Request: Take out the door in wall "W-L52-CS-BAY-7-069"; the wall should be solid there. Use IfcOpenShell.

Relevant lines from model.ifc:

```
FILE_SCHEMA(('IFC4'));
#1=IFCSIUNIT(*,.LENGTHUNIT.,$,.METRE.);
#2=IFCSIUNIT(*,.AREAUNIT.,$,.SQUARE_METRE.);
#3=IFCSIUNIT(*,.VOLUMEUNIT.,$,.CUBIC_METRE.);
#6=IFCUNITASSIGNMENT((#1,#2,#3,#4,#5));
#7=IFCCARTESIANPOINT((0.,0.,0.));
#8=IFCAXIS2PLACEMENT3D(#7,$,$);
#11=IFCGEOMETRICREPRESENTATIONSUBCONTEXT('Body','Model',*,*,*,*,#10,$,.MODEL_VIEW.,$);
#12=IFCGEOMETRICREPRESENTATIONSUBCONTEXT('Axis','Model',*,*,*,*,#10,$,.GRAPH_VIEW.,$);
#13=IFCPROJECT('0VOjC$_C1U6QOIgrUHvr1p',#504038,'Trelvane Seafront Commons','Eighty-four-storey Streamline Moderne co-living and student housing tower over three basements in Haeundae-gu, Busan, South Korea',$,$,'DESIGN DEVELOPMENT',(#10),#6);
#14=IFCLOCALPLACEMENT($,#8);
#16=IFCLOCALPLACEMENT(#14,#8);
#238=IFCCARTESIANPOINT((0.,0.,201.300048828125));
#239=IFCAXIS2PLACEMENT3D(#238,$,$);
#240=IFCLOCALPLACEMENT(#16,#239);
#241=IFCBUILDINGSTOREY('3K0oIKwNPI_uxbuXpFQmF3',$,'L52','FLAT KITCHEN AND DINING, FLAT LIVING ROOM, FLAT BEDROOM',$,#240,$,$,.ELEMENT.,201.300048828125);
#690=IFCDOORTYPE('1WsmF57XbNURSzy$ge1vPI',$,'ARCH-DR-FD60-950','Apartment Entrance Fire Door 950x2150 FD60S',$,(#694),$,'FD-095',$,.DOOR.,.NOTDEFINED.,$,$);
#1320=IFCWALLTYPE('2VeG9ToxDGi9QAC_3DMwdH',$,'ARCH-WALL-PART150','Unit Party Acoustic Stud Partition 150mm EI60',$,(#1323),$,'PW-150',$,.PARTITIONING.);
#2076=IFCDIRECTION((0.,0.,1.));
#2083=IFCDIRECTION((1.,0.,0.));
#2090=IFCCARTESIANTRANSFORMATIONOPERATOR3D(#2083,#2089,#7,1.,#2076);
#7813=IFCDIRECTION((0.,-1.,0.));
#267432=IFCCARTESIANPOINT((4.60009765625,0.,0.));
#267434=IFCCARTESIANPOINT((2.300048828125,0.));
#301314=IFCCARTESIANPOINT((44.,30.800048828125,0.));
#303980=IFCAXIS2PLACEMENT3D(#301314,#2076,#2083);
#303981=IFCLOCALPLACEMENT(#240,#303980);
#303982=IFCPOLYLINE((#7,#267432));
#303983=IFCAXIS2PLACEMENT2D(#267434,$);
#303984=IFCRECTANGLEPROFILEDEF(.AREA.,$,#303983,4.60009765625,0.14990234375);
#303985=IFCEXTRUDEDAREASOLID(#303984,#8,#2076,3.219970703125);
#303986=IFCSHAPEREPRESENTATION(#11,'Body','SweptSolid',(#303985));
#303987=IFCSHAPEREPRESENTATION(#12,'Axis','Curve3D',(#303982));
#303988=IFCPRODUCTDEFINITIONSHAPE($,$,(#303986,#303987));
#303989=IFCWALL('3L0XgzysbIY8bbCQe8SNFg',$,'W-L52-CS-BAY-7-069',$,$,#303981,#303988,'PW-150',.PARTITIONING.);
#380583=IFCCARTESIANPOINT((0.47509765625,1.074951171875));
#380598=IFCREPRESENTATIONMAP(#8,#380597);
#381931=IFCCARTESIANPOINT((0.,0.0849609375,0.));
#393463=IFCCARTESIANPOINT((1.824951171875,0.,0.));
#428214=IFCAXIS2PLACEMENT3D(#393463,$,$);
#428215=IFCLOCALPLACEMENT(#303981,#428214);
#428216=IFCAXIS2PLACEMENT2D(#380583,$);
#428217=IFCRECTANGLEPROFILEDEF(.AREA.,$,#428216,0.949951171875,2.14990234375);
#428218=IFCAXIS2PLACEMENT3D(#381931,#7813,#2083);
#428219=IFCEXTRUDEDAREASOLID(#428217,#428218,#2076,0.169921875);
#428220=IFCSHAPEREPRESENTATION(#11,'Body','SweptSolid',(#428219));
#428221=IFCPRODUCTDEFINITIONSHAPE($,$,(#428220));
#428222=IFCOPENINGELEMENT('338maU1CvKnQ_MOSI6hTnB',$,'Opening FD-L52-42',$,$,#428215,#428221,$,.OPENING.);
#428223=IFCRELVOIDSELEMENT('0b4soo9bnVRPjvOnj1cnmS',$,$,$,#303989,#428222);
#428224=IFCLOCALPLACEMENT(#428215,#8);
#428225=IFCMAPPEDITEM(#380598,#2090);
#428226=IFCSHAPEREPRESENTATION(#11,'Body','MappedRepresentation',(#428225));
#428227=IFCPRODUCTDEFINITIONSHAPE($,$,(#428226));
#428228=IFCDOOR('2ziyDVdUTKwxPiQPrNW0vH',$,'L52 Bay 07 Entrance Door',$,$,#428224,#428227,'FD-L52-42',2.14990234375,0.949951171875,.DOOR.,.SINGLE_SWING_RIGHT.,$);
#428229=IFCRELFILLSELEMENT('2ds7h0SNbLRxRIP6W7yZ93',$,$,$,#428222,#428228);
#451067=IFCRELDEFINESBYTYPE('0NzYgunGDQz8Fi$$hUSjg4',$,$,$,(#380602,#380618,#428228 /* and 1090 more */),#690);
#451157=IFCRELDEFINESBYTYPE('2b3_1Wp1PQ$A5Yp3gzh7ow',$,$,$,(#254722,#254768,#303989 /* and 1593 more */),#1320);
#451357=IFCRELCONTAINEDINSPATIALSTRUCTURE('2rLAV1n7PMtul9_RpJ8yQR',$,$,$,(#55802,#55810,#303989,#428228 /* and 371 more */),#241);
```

```python
import ifcopenshell
import ifcopenshell.api.feature
import ifcopenshell.api.root
import ifcopenshell.geom
import ifcopenshell.util.shape

model = ifcopenshell.open("model.ifc")
settings = ifcopenshell.geom.settings()


def volume(element):
    """Net volume in cubic metres, openings subtracted."""
    shape = ifcopenshell.geom.create_shape(settings, element)
    return ifcopenshell.util.shape.get_volume(shape.geometry)


door = model.by_guid("2ziyDVdUTKwxPiQPrNW0vH")
opening = door.FillsVoids[0].RelatingOpeningElement
wall = opening.VoidsElements[0].RelatingBuildingElement
before = volume(wall)

ifcopenshell.api.root.remove_product(model, product=door)
ifcopenshell.api.feature.remove_feature(model, feature=opening)

after = volume(wall)

print(f"wall volume {before:.3f} -> {after:.3f} m3")

model.write("model_rev.ifc")
```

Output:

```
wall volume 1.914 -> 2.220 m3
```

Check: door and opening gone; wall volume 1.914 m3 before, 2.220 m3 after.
